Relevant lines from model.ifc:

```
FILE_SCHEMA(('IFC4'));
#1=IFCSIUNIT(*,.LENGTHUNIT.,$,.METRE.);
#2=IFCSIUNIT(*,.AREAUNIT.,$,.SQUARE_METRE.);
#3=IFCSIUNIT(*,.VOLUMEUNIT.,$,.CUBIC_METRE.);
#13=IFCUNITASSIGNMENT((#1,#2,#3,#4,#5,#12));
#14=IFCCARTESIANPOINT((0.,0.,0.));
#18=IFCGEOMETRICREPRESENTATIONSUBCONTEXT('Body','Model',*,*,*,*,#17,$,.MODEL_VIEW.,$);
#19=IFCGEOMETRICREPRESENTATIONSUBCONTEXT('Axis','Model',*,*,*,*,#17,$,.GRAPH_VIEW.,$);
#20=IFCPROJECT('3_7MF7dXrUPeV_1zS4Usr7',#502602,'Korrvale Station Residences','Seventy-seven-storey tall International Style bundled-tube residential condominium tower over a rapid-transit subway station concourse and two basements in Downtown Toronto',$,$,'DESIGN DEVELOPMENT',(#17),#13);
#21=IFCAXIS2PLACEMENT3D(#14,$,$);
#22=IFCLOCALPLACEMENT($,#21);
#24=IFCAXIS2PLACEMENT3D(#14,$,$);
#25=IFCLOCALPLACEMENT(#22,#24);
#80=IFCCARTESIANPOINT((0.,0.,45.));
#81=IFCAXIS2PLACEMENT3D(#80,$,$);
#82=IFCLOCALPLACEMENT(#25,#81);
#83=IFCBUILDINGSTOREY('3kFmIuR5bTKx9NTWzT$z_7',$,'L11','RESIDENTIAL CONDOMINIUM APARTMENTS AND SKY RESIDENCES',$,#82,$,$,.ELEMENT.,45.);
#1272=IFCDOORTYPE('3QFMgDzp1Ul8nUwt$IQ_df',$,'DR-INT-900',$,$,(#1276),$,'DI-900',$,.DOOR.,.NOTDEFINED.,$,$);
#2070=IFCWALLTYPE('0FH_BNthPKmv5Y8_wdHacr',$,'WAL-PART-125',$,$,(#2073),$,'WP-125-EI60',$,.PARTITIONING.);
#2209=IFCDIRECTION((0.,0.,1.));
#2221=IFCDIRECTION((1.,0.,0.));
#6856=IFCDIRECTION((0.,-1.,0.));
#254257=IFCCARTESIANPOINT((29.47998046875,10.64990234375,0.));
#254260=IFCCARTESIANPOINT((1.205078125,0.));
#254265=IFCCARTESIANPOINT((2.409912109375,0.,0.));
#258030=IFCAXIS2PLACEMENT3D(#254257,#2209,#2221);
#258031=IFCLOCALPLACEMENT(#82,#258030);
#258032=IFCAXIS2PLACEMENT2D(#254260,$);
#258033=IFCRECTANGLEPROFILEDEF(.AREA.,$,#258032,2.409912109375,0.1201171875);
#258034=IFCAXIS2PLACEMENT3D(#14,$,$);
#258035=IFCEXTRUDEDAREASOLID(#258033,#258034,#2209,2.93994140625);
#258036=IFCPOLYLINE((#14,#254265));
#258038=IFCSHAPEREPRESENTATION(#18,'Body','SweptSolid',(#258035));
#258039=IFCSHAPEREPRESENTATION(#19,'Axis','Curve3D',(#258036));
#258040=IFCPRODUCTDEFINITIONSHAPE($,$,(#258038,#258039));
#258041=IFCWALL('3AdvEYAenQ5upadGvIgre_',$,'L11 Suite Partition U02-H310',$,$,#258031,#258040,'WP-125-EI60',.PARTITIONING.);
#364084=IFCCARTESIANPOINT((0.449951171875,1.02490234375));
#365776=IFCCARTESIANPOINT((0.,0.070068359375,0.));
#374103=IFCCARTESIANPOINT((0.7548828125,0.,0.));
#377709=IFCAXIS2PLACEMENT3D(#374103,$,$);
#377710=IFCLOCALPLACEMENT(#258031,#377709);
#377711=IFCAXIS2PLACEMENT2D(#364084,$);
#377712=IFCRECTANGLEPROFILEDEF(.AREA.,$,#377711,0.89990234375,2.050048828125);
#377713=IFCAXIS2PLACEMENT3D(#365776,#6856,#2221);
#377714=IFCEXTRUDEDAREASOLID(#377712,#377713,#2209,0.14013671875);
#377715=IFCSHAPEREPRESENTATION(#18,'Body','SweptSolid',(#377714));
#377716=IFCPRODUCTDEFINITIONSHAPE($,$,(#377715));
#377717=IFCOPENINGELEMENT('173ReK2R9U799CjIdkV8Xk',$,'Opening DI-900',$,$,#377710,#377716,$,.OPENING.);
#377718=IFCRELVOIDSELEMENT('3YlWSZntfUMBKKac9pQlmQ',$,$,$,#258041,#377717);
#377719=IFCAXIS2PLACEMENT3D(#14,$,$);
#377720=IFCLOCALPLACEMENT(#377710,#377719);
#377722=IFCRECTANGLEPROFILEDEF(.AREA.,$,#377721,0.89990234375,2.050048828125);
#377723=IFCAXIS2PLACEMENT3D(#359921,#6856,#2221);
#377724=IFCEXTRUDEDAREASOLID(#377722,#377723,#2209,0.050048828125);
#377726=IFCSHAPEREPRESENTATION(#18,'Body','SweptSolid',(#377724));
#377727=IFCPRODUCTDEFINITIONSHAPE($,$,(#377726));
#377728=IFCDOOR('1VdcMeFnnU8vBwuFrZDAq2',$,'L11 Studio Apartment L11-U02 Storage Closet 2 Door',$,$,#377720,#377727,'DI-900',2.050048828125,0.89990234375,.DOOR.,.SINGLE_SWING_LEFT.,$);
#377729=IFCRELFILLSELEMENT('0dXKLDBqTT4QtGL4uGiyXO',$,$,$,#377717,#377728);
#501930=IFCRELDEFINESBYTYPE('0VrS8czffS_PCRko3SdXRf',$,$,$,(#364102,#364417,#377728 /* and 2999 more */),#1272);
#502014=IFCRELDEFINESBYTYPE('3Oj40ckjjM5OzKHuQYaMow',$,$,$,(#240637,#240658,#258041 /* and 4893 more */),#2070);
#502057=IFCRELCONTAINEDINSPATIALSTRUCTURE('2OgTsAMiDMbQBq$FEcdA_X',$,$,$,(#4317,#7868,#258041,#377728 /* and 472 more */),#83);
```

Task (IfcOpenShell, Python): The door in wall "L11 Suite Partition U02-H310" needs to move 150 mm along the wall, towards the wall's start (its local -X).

```python
import ifcopenshell
import ifcopenshell.api.geometry
import ifcopenshell.util.placement

model = ifcopenshell.open("model.ifc")

door = model.by_guid("1VdcMeFnnU8vBwuFrZDAq2")
opening = door.FillsVoids[0].RelatingOpeningElement
wall = opening.VoidsElements[0].RelatingBuildingElement

wall_matrix = ifcopenshell.util.placement.get_local_placement(wall.ObjectPlacement)
shift = wall_matrix[:3, 0] * -0.15
before = ifcopenshell.util.placement.get_local_placement(door.ObjectPlacement)[:3, 3].copy()

# The door is placed relative to its opening, so it follows when the opening moves.
matrix = ifcopenshell.util.placement.get_local_placement(opening.ObjectPlacement)
matrix[:3, 3] += shift
ifcopenshell.api.geometry.edit_object_placement(
    model, product=opening, matrix=matrix, is_si=False, should_transform_children=True
)

after = ifcopenshell.util.placement.get_local_placement(door.ObjectPlacement)[:3, 3]
print("door moved by", (after - before).round(3) + 0.0)

model.write("model_updated.ifc")
```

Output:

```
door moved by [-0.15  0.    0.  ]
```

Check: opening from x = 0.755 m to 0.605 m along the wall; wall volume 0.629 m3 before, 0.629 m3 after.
